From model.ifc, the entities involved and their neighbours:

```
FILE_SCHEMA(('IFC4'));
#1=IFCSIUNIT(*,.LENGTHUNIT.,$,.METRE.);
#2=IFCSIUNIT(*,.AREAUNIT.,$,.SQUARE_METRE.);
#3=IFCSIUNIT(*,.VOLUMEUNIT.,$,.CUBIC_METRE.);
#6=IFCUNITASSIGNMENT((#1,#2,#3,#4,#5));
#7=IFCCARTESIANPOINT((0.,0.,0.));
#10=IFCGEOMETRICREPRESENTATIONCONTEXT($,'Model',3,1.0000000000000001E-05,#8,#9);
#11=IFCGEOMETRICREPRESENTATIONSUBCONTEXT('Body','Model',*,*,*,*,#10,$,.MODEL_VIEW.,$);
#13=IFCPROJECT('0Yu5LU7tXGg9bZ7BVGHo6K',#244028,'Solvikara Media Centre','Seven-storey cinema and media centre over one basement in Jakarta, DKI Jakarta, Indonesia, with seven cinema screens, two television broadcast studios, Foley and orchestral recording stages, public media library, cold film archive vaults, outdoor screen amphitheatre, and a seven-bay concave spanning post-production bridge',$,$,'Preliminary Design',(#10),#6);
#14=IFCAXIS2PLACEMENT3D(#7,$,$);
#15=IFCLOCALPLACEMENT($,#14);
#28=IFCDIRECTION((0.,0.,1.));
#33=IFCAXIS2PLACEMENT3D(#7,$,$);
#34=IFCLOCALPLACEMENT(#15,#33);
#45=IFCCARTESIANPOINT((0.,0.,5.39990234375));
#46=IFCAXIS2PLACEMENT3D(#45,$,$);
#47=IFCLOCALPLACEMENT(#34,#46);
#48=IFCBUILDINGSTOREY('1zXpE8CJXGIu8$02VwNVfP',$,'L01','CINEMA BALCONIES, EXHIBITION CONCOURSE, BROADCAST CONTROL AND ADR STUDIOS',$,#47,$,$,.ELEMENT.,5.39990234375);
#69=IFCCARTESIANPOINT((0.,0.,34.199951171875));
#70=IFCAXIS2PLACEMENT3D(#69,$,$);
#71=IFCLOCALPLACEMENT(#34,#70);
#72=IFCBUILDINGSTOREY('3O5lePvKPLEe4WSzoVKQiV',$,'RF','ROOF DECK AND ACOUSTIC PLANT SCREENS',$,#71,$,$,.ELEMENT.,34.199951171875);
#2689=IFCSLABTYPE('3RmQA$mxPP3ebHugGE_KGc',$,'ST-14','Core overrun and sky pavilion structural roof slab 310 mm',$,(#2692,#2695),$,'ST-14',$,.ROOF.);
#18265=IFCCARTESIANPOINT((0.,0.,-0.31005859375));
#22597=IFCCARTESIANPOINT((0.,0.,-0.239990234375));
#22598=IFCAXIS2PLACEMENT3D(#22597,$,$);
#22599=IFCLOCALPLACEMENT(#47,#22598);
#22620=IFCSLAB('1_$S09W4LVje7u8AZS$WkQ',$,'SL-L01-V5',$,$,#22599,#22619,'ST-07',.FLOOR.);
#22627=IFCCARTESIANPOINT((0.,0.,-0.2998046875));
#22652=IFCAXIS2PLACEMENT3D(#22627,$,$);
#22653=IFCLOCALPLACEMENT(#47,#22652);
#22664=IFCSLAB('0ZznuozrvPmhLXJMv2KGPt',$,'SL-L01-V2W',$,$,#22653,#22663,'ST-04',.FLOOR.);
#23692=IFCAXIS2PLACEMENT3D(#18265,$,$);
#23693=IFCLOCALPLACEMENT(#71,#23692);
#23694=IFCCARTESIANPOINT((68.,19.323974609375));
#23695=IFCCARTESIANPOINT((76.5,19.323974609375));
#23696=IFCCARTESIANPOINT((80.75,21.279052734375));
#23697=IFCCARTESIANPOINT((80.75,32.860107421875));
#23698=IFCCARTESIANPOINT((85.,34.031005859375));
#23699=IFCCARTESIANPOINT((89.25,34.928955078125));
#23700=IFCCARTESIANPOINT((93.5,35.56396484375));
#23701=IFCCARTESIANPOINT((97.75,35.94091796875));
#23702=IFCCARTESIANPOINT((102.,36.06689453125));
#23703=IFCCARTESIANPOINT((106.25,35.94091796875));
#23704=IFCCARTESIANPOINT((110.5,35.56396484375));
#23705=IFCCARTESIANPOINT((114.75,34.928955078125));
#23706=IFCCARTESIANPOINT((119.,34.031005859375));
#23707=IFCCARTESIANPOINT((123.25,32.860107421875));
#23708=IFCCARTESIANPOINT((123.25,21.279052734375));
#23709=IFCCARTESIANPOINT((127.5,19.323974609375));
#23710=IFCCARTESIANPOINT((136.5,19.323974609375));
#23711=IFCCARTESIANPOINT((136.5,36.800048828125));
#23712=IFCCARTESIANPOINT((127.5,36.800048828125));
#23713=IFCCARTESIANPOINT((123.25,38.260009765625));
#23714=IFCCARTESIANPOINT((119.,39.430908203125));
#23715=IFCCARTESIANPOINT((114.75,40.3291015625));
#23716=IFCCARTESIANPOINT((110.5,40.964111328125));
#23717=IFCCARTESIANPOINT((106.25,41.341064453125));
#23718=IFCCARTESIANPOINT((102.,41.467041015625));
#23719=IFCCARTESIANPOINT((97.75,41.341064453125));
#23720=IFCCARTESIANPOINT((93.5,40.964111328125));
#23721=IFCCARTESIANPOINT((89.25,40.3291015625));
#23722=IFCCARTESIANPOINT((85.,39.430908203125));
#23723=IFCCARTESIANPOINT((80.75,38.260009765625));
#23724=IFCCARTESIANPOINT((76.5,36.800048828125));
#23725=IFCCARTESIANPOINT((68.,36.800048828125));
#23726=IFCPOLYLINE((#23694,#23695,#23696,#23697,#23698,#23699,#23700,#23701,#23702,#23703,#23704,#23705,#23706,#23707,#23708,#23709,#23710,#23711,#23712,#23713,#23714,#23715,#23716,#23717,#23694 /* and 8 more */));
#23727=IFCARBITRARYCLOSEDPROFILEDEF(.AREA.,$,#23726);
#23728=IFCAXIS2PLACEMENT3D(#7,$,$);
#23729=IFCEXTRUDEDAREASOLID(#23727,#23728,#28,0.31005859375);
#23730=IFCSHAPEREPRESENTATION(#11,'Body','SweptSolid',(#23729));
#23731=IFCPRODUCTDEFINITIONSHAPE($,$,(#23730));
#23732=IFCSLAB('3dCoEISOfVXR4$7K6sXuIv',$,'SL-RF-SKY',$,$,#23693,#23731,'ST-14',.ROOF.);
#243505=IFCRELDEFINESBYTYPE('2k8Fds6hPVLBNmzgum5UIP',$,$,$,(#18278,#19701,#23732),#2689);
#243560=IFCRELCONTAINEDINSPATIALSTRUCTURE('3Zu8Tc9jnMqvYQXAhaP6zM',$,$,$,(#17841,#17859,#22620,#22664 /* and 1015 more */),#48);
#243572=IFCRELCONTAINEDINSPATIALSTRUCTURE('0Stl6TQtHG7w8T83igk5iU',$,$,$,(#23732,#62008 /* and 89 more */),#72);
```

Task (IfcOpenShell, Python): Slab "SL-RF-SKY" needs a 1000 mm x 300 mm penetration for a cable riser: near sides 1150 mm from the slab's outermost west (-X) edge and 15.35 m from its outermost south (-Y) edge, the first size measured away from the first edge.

```python
import numpy as np
import ifcopenshell
import ifcopenshell.api.feature
import ifcopenshell.api.geometry
import ifcopenshell.api.root
import ifcopenshell.geom
import ifcopenshell.util.placement
import ifcopenshell.util.representation
import ifcopenshell.util.shape
import ifcopenshell.util.unit

model = ifcopenshell.open("model.ifc")
unit_scale = ifcopenshell.util.unit.calculate_unit_scale(model)
settings = ifcopenshell.geom.settings()


def volume(element):
    """Net volume in cubic metres, openings subtracted."""
    shape = ifcopenshell.geom.create_shape(settings, element)
    return ifcopenshell.util.shape.get_volume(shape.geometry)


slab = model.by_id(23732)
before = volume(slab)

# Extent in the slab's own axes, in metres. The edges named are its -X and -Y sides.
slab_shape = ifcopenshell.geom.create_shape(settings, slab)
vertices = ifcopenshell.util.shape.get_vertices(slab_shape.geometry)
x_min, y_min, bottom = vertices.min(axis=0)
top = vertices[:, 2].max()

opening = ifcopenshell.api.root.create_entity(model, ifc_class="IfcOpeningElement", name="Cable riser opening", predefined_type="OPENING")
context = ifcopenshell.util.representation.get_context(model, "Model", "Body", "MODEL_VIEW")
width, depth = 1, 0.3
outline = [(0.0, 0.0), (width, 0.0), (width, depth), (0.0, depth), (0.0, 0.0)]
# Overshoot both faces by 50 mm so the cut is clean.
shape = ifcopenshell.api.geometry.add_slab_representation(
    model, context=context, depth=top - bottom + 0.1, polyline=outline
)
ifcopenshell.api.geometry.assign_representation(model, product=opening, representation=shape)

matrix = ifcopenshell.util.placement.get_local_placement(slab.ObjectPlacement)
matrix[:, 3] = matrix @ np.append(np.array([x_min + 1.15, y_min + 15.35, bottom - 0.05]) / unit_scale, 1.0)
ifcopenshell.api.geometry.edit_object_placement(model, product=opening, matrix=matrix, is_si=False)
ifcopenshell.api.feature.add_feature(model, feature=opening, element=slab)

after = volume(slab)

print(f"slab volume {before:.3f} -> {after:.3f} m3")

model.write("model_edited.ifc")
```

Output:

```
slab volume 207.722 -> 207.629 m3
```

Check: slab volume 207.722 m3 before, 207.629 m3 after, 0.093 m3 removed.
